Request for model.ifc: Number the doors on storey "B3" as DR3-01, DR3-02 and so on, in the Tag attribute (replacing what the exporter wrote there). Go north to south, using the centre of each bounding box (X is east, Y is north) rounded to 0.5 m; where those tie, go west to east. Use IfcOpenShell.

First a look at what the model holds.

```python
import ifcopenshell
import ifcopenshell.util.element
import ifcopenshell.util.placement

model = ifcopenshell.open("model.ifc")
print(model.schema)
storey = next(s for s in model.by_type("IfcBuildingStorey") if s.Name == "B3")
doors = [e for e in ifcopenshell.util.element.get_decomposition(storey) if e.is_a("IfcDoor")]
for e in sorted(doors, key=lambda e: e.id()):
    origin = ifcopenshell.util.placement.get_local_placement(e.ObjectPlacement)[:3, 3]
    print(e.id(), e.Tag, e.Name, origin.round(2) + 0.0, sep=" | ")
```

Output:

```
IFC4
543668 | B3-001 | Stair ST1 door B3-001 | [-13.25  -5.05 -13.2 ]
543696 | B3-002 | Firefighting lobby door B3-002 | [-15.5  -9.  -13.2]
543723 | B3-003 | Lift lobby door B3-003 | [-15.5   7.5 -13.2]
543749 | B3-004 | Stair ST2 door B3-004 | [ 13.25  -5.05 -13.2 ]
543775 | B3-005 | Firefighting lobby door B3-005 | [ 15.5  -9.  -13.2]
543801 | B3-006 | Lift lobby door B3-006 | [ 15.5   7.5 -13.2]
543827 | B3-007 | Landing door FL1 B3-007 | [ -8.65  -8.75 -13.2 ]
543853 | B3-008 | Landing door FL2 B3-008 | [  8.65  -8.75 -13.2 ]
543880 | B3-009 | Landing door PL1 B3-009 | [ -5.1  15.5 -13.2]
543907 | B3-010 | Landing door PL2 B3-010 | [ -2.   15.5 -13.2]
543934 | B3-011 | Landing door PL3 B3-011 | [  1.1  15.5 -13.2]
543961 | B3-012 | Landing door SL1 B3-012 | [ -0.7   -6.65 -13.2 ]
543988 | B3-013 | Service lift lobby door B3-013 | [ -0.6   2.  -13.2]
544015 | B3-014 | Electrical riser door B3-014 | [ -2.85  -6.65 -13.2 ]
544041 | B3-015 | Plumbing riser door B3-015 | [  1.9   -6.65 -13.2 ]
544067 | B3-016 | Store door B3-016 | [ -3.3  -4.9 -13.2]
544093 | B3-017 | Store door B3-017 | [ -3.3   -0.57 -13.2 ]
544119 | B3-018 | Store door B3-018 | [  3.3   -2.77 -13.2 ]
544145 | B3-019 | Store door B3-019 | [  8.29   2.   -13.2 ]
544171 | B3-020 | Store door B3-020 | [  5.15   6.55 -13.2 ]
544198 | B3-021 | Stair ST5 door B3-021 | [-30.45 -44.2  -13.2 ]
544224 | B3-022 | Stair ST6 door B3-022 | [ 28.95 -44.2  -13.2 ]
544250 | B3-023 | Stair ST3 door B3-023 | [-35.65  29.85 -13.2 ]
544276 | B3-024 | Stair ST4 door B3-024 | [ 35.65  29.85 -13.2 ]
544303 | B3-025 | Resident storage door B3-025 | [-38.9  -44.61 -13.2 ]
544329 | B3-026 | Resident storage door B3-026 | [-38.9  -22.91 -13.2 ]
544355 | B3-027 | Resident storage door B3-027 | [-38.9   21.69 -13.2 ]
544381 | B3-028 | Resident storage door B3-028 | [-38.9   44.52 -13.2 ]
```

```python
import ifcopenshell
import ifcopenshell.geom
import ifcopenshell.util.element
import ifcopenshell.util.shape

model = ifcopenshell.open("model.ifc")
settings = ifcopenshell.geom.settings()
settings.set("use-world-coords", True)


def centre(element):
    shape = ifcopenshell.geom.create_shape(settings, element)
    return ifcopenshell.util.shape.get_bbox_centroid(shape.geometry)


storey = next(s for s in model.by_type("IfcBuildingStorey") if s.Name == "B3")
doors = [e for e in ifcopenshell.util.element.get_decomposition(storey) if e.is_a("IfcDoor")]

# Insertion points can sit at a corner or the storey origin, so sort by the geometry (in metres).
centres = {e: centre(e) for e in doors}
doors.sort(key=lambda e: (-round(centres[e][1] / 0.5), centres[e][0]))

for i, e in enumerate(doors, start=1):
    number = f"DR3-{i:02d}"
    e.Tag = number
    print(e.id(), number)

model.write("model_updated.ifc")
```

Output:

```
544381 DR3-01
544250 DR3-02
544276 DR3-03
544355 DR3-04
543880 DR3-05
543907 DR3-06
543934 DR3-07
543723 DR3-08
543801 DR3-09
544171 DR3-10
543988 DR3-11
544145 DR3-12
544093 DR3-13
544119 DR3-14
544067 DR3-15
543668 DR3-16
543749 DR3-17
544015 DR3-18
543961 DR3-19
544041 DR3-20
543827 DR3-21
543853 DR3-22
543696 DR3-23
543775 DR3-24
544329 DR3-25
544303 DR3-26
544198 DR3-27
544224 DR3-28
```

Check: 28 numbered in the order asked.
